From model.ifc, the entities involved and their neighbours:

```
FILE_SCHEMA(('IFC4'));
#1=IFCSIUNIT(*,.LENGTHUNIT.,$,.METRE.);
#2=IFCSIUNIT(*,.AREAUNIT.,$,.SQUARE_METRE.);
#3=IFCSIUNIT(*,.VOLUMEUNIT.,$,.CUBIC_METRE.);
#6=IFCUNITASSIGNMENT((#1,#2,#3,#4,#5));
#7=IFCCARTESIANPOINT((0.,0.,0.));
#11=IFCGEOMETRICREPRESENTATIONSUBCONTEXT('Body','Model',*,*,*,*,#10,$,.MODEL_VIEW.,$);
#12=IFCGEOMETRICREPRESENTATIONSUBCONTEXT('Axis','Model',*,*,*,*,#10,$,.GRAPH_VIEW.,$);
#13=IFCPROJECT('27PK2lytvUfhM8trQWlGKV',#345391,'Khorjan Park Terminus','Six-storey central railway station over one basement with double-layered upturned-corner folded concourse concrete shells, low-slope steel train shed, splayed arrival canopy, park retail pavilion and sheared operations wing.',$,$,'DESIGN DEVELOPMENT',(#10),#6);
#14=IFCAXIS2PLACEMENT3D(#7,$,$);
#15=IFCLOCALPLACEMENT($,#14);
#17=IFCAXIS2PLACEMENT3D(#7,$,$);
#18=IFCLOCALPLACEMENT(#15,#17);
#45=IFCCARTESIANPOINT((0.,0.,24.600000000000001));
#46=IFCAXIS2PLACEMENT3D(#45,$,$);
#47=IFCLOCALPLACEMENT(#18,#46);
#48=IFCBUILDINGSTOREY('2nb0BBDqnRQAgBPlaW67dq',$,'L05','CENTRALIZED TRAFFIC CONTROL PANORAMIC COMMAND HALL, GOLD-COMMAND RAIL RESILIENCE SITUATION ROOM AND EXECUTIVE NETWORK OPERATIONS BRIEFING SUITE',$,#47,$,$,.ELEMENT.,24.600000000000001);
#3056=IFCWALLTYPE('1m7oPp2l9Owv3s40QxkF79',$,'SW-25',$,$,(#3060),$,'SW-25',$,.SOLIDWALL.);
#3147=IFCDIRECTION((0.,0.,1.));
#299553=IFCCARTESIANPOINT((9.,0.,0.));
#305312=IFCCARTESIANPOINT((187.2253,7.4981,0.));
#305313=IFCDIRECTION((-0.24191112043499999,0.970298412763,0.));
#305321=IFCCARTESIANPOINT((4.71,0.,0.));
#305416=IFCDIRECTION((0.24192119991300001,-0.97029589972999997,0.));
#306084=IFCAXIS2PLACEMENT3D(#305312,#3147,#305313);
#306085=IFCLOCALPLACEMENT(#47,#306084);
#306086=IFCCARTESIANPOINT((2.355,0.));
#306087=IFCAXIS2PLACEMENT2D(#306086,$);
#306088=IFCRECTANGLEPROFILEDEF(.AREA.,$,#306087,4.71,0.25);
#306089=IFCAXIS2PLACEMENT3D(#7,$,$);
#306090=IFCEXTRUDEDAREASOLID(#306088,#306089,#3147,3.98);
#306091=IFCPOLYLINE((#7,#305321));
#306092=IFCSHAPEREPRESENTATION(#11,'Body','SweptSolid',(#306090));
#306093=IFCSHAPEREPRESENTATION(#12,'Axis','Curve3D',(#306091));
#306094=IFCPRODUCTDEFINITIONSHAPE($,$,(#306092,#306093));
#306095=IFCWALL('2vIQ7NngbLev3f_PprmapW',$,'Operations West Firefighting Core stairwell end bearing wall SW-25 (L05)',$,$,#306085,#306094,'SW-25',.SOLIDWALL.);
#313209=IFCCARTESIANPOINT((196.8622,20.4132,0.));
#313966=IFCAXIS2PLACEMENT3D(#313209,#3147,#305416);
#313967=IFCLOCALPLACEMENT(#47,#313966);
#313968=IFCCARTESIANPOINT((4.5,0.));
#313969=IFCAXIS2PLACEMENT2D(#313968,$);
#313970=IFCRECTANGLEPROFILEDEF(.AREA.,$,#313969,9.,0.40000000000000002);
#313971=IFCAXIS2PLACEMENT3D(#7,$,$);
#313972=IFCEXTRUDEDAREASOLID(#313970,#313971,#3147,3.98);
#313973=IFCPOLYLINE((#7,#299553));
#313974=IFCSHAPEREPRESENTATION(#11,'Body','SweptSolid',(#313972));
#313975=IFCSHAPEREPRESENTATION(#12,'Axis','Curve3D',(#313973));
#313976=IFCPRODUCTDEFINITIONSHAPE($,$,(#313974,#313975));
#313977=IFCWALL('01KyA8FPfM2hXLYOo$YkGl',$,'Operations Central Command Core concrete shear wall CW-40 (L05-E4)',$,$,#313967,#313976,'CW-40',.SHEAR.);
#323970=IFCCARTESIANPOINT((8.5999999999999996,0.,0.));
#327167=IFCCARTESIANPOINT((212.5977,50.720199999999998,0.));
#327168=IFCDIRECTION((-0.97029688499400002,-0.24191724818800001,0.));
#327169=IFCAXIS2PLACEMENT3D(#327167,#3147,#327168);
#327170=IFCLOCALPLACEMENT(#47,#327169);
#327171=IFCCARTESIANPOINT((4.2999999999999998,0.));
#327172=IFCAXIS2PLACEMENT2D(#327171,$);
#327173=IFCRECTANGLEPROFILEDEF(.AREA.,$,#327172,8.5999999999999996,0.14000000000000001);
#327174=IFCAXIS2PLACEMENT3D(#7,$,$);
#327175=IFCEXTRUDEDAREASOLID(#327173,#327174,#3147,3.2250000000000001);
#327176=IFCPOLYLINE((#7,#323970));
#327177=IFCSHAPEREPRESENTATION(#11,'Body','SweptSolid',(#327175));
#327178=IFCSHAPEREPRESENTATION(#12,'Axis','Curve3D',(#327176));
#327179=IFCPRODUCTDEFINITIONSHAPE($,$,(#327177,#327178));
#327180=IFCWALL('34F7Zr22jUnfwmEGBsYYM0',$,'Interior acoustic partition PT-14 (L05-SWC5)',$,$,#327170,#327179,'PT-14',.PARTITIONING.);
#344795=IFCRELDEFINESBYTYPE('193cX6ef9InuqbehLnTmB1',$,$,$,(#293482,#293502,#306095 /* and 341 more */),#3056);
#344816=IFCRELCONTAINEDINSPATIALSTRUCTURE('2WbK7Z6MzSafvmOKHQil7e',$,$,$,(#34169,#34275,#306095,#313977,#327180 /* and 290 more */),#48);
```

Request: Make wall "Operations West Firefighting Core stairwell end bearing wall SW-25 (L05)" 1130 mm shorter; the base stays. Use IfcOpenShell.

```python
import ifcopenshell
import ifcopenshell.geom
import ifcopenshell.util.representation
import ifcopenshell.util.shape
import ifcopenshell.util.unit

model = ifcopenshell.open("model.ifc")
unit_scale = ifcopenshell.util.unit.calculate_unit_scale(model)
settings = ifcopenshell.geom.settings()


def volume(element):
    """Net volume in cubic metres, openings subtracted."""
    shape = ifcopenshell.geom.create_shape(settings, element)
    return ifcopenshell.util.shape.get_volume(shape.geometry)


wall = model.by_guid("2vIQ7NngbLev3f_PprmapW")
before = volume(wall)

body = ifcopenshell.util.representation.get_representation(wall, "Model", "Body")
solid = body.Items[0]
old_height = solid.Depth
solid.Depth -= 1.13 / unit_scale
after = volume(wall)

print(f"height {old_height:g} -> {solid.Depth:g}, volume {before:.3f} -> {after:.3f} m3")

model.write("model_updated.ifc")
```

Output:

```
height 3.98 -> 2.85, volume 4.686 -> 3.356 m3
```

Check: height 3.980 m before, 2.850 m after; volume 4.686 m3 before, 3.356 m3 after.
